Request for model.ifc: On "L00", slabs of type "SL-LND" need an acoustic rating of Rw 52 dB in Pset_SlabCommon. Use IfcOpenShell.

First a look at what the model holds.

```python
import ifcopenshell
import ifcopenshell.util.element

model = ifcopenshell.open("model.ifc")
print(model.schema)
storey = next(s for s in model.by_type("IfcBuildingStorey") if s.Name == "L00")
slabs = [e for e in ifcopenshell.util.element.get_decomposition(storey) if e.is_a("IfcSlab")]
seen = {}
for e in slabs:
    element_type = ifcopenshell.util.element.get_type(e)
    key = (element_type.Name if element_type != e and element_type else None, ifcopenshell.util.element.get_pset(e, "Pset_SlabCommon", "AcousticRating"))
    seen[key] = seen.get(key, 0) + 1
for (name, value), count in sorted(seen.items(), key=str):
    print(count, "x", name, "|", value)
```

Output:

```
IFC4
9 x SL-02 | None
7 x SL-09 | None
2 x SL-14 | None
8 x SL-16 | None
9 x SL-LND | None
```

```python
import ifcopenshell
import ifcopenshell.api.pset
import ifcopenshell.util.element

model = ifcopenshell.open("model.ifc")

storey = next(s for s in model.by_type("IfcBuildingStorey") if s.Name == "L00")
slabs = [e for e in ifcopenshell.util.element.get_decomposition(storey) if e.is_a("IfcSlab")]

count = 0
for e in slabs:
    element_type = ifcopenshell.util.element.get_type(e)
    if element_type in (None, e) or element_type.Name != "SL-LND":
        continue
    # add_pset returns the element's existing set when there is one.
    pset = ifcopenshell.api.pset.add_pset(model, product=e, name="Pset_SlabCommon")
    ifcopenshell.api.pset.edit_pset(model, pset=pset, properties={"AcousticRating": "Rw 52 dB"})
    count += 1

print(count, "slabs updated")

model.write("model_rev.ifc")
```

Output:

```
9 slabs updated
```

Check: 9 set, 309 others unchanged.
